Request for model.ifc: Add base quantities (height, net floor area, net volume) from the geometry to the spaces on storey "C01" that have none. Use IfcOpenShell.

First a look at what the model holds.

```python
import ifcopenshell
import ifcopenshell.util.element
import ifcopenshell.util.unit

model = ifcopenshell.open("model.ifc")
print(model.schema)
for unit_type in ("LENGTHUNIT", "AREAUNIT", "VOLUMEUNIT"):
    print(unit_type, ifcopenshell.util.unit.calculate_unit_scale(model, unit_type))
storey = next(s for s in model.by_type("IfcBuildingStorey") if s.Name == "C01")
spaces = [e for e in ifcopenshell.util.element.get_decomposition(storey) if e.is_a("IfcSpace")]
for e in sorted(spaces, key=lambda e: e.id()):
    print(e.id(), e.is_a(), e.Name, list(ifcopenshell.util.element.get_psets(e, qtos_only=True)), sep=" | ")
```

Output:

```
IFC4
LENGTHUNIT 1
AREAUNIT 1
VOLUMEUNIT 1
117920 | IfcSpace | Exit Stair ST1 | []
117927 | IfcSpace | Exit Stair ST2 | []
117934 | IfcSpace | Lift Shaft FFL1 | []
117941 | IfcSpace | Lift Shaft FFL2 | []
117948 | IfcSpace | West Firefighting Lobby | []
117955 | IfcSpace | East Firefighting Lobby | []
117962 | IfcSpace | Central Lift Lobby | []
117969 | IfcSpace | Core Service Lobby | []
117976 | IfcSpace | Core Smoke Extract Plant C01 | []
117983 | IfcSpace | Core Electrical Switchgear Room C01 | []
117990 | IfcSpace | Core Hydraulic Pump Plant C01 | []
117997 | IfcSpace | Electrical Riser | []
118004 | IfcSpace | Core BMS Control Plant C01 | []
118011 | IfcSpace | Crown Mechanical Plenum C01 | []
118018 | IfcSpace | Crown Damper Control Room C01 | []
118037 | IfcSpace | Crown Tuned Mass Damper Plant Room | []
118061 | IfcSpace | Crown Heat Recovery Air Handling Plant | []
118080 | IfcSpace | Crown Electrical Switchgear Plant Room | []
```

```python
import ifcopenshell
import ifcopenshell.api.pset
import ifcopenshell.geom
import ifcopenshell.util.element
import ifcopenshell.util.shape
import ifcopenshell.util.unit

model = ifcopenshell.open("model.ifc")
unit_scale = ifcopenshell.util.unit.calculate_unit_scale(model)
area_scale = ifcopenshell.util.unit.calculate_unit_scale(model, "AREAUNIT")
volume_scale = ifcopenshell.util.unit.calculate_unit_scale(model, "VOLUMEUNIT")
settings = ifcopenshell.geom.settings()

storey = next(s for s in model.by_type("IfcBuildingStorey") if s.Name == "C01")
spaces = [e for e in ifcopenshell.util.element.get_decomposition(storey) if e.is_a("IfcSpace")]

for e in sorted(spaces, key=lambda e: e.id()):
    if ifcopenshell.util.element.get_psets(e, qtos_only=True, should_inherit=False):
        continue
    # Geometry comes back in metres, in the element's own axes.
    shape = ifcopenshell.geom.create_shape(settings, e)
    values = {
        "Height": ifcopenshell.util.shape.get_z(shape.geometry) / unit_scale,
        "NetFloorArea": ifcopenshell.util.shape.get_footprint_area(shape.geometry) / area_scale,
        "NetVolume": ifcopenshell.util.shape.get_volume(shape.geometry) / volume_scale,
    }
    qto = ifcopenshell.api.pset.add_qto(model, product=e, name="Qto_SpaceBaseQuantities")
    ifcopenshell.api.pset.edit_qto(model, qto=qto, properties=values)
    print(e.id(), {k: round(v, 3) for k, v in values.items()})

model.write("model-out.ifc")
```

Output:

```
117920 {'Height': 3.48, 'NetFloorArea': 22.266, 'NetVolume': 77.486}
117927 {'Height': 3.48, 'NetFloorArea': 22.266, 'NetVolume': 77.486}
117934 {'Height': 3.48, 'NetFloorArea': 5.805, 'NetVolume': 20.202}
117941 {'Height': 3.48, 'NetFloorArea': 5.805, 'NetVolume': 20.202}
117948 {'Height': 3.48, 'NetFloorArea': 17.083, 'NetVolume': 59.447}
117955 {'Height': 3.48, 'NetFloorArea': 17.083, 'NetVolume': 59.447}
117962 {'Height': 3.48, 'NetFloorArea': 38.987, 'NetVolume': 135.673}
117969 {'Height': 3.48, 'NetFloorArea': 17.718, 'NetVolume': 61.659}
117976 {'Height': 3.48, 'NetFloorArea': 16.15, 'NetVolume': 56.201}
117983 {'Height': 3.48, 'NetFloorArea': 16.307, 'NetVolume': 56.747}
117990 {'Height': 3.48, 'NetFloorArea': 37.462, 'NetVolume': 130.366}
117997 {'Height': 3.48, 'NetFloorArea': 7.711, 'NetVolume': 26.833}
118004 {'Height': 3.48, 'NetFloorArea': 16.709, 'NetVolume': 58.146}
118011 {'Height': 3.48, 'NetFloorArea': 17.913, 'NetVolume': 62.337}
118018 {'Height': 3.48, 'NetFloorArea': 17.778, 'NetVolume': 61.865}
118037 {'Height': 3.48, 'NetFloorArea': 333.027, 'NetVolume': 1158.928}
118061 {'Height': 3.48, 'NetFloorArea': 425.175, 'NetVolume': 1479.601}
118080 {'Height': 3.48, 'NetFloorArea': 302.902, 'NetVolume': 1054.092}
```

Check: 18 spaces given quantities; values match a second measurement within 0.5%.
